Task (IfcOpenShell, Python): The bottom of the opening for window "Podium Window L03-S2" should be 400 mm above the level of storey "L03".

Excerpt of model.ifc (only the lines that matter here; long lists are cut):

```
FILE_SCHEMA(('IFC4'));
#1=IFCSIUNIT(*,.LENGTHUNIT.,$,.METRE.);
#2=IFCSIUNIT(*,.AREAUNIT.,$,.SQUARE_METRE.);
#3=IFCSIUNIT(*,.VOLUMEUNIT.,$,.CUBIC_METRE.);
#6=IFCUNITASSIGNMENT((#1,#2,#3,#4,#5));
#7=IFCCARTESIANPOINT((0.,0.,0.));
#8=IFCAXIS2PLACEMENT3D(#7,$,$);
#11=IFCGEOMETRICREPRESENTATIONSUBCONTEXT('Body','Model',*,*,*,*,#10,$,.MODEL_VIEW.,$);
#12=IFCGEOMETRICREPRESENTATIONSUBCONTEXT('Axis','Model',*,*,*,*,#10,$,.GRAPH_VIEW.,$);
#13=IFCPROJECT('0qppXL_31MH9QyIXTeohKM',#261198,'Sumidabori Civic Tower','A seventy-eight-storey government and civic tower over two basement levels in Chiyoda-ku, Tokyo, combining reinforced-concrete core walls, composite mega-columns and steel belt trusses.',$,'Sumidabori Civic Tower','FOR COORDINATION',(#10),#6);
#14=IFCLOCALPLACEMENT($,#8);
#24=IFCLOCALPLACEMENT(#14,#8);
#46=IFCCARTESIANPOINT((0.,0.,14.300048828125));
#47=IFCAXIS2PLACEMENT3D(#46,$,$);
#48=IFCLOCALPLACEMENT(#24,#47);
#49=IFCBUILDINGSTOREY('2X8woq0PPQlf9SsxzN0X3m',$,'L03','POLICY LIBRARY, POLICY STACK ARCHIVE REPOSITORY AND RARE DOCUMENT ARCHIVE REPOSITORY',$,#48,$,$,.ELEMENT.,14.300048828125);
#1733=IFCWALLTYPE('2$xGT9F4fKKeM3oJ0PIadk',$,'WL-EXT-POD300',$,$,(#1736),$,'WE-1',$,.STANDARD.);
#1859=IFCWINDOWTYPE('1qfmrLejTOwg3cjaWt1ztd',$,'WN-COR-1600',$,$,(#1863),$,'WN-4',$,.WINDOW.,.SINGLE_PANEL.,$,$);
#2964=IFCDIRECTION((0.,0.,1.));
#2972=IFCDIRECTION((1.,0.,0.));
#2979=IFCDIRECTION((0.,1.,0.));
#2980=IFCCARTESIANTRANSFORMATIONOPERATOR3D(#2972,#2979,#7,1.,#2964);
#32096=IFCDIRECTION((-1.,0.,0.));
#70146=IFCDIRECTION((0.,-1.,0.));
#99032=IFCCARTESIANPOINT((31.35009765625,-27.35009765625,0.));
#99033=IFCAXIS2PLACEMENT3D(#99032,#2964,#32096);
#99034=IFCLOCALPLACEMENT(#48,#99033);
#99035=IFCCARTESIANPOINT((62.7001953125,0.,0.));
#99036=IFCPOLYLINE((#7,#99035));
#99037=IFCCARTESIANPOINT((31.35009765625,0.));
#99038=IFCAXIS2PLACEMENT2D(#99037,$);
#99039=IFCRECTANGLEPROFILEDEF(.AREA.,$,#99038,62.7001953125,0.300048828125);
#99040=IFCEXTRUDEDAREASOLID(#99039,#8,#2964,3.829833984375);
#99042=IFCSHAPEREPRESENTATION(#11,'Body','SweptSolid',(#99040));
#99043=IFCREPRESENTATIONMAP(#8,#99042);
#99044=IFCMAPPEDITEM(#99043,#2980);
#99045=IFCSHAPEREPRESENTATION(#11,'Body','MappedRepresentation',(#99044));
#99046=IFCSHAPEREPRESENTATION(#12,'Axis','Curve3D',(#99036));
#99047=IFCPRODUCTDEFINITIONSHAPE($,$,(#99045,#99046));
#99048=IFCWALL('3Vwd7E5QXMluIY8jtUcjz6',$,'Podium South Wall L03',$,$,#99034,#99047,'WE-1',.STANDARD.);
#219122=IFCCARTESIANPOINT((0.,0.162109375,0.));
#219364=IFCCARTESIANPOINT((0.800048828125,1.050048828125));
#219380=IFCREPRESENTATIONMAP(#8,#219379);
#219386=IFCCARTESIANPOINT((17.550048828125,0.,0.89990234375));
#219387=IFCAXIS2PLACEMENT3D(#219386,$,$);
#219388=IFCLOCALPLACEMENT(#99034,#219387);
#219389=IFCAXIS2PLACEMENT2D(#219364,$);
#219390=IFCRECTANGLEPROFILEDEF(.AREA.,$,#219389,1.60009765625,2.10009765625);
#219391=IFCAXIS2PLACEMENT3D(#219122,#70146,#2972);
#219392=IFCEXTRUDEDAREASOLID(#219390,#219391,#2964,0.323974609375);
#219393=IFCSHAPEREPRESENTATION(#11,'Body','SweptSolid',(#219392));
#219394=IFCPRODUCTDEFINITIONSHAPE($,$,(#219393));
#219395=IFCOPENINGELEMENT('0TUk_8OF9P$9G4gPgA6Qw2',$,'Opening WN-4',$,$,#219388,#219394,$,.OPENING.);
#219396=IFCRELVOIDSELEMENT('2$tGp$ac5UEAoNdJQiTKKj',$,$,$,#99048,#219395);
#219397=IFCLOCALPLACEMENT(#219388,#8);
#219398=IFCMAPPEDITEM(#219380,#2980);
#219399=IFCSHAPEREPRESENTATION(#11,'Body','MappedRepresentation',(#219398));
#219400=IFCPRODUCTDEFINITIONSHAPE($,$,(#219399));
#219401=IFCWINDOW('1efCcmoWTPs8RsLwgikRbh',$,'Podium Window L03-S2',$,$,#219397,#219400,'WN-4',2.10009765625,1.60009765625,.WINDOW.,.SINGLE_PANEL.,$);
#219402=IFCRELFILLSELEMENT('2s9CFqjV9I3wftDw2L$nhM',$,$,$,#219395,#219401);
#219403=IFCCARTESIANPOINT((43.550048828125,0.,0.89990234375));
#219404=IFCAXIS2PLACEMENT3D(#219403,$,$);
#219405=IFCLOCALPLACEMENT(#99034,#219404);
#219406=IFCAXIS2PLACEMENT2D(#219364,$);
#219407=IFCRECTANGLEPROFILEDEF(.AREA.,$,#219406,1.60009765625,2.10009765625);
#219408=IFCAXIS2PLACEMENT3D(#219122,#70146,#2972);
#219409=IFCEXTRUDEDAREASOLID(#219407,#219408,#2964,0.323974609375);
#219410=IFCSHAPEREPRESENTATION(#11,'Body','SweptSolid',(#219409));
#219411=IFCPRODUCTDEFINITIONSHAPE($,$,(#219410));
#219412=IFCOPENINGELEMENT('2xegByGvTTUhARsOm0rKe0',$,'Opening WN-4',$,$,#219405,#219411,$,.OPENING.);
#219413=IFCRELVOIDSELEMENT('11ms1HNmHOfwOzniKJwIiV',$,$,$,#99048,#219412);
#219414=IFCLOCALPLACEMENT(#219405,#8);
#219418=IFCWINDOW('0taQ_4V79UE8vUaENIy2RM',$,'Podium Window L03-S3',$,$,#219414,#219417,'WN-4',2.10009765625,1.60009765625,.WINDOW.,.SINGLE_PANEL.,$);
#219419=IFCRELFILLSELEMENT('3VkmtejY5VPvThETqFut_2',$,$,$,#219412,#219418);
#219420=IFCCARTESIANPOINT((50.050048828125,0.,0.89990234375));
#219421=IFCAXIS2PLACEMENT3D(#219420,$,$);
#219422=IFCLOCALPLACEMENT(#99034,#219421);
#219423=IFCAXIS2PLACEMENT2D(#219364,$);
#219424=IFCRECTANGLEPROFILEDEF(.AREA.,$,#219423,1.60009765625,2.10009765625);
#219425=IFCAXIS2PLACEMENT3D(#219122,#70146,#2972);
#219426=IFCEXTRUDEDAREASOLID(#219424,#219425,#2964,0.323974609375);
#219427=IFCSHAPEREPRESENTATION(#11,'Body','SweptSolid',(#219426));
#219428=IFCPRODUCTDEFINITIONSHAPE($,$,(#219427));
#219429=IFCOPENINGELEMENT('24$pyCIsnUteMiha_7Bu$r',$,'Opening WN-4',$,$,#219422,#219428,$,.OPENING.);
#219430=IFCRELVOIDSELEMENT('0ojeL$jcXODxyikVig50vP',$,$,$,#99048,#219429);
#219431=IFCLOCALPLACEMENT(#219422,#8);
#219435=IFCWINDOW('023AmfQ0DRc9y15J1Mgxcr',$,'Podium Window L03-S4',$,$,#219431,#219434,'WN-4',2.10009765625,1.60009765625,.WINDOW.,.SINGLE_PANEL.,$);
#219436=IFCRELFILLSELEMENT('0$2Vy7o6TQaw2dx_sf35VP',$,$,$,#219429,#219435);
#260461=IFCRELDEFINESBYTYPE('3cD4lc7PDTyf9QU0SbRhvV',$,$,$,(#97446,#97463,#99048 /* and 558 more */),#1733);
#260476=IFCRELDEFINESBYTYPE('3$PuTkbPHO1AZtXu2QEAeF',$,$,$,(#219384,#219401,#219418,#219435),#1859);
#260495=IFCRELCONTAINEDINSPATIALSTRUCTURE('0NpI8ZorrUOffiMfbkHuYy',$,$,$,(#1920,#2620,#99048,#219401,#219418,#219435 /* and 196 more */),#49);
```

```python
import numpy as np
import ifcopenshell
import ifcopenshell.api.geometry
import ifcopenshell.geom
import ifcopenshell.util.element
import ifcopenshell.util.placement
import ifcopenshell.util.shape
import ifcopenshell.util.unit

model = ifcopenshell.open("model.ifc")
unit_scale = ifcopenshell.util.unit.calculate_unit_scale(model)

window = model.by_id(219401)
opening = window.FillsVoids[0].RelatingOpeningElement
storey = ifcopenshell.util.element.get_container(window, ifc_class="IfcBuildingStorey")
level = ifcopenshell.util.placement.get_local_placement(storey.ObjectPlacement)[2, 3]

# The opening's origin need not be at the sill, so measure its lowest point.
shape = ifcopenshell.geom.create_shape(ifcopenshell.geom.settings(), opening)
bottom = ifcopenshell.util.shape.get_shape_bottom_elevation(shape, shape.geometry) / unit_scale
dz = level + 0.4 / unit_scale - bottom

shift = np.array([0.0, 0.0, dz])
# The window is placed relative to its opening, so it follows when the opening moves.
matrix = ifcopenshell.util.placement.get_local_placement(opening.ObjectPlacement)
matrix[:3, 3] += shift
ifcopenshell.api.geometry.edit_object_placement(
    model, product=opening, matrix=matrix, is_si=False, should_transform_children=True
)

print(f"moved by {dz * unit_scale:+.3f} m")

model.write("model-out.ifc")
```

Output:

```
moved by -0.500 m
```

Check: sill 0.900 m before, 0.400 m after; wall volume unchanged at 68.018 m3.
